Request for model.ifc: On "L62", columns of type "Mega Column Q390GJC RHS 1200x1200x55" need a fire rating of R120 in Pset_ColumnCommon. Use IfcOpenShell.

First a look at what the model holds.

```python
import ifcopenshell
import ifcopenshell.util.element

model = ifcopenshell.open("model.ifc")
print(model.schema)
storey = next(s for s in model.by_type("IfcBuildingStorey") if s.Name == "L62")
columns = [e for e in ifcopenshell.util.element.get_decomposition(storey) if e.is_a("IfcColumn")]
seen = {}
for e in columns:
    element_type = ifcopenshell.util.element.get_type(e)
    key = (element_type.Name if element_type != e and element_type else None, ifcopenshell.util.element.get_pset(e, "Pset_ColumnCommon", "FireRating"))
    seen[key] = seen.get(key, 0) + 1
for (name, value), count in sorted(seen.items(), key=str):
    print(count, "x", name, "|", value)
```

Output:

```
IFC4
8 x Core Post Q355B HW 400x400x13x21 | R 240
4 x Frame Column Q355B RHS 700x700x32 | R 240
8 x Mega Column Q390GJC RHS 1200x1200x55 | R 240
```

```python
import ifcopenshell
import ifcopenshell.api.pset
import ifcopenshell.util.element

model = ifcopenshell.open("model.ifc")

storey = next(s for s in model.by_type("IfcBuildingStorey") if s.Name == "L62")
columns = [e for e in ifcopenshell.util.element.get_decomposition(storey) if e.is_a("IfcColumn")]

count = 0
for e in columns:
    element_type = ifcopenshell.util.element.get_type(e)
    if element_type in (None, e) or element_type.Name != "Mega Column Q390GJC RHS 1200x1200x55":
        continue
    found = ifcopenshell.util.element.get_pset(e, "Pset_ColumnCommon", should_inherit=False)
    if found:
        pset = model.by_id(found["id"])
        if len(ifcopenshell.util.element.get_elements_by_pset(pset)) > 1:
            pset = ifcopenshell.api.pset.unshare_pset(model, products=[e], pset=pset)[0]
    else:
        pset = ifcopenshell.api.pset.add_pset(model, product=e, name="Pset_ColumnCommon")
    ifcopenshell.api.pset.edit_pset(model, pset=pset, properties={"FireRating": "R120"})
    count += 1

print(count, "columns updated")

model.write("model-out.ifc")
```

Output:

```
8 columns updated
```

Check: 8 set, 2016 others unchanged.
